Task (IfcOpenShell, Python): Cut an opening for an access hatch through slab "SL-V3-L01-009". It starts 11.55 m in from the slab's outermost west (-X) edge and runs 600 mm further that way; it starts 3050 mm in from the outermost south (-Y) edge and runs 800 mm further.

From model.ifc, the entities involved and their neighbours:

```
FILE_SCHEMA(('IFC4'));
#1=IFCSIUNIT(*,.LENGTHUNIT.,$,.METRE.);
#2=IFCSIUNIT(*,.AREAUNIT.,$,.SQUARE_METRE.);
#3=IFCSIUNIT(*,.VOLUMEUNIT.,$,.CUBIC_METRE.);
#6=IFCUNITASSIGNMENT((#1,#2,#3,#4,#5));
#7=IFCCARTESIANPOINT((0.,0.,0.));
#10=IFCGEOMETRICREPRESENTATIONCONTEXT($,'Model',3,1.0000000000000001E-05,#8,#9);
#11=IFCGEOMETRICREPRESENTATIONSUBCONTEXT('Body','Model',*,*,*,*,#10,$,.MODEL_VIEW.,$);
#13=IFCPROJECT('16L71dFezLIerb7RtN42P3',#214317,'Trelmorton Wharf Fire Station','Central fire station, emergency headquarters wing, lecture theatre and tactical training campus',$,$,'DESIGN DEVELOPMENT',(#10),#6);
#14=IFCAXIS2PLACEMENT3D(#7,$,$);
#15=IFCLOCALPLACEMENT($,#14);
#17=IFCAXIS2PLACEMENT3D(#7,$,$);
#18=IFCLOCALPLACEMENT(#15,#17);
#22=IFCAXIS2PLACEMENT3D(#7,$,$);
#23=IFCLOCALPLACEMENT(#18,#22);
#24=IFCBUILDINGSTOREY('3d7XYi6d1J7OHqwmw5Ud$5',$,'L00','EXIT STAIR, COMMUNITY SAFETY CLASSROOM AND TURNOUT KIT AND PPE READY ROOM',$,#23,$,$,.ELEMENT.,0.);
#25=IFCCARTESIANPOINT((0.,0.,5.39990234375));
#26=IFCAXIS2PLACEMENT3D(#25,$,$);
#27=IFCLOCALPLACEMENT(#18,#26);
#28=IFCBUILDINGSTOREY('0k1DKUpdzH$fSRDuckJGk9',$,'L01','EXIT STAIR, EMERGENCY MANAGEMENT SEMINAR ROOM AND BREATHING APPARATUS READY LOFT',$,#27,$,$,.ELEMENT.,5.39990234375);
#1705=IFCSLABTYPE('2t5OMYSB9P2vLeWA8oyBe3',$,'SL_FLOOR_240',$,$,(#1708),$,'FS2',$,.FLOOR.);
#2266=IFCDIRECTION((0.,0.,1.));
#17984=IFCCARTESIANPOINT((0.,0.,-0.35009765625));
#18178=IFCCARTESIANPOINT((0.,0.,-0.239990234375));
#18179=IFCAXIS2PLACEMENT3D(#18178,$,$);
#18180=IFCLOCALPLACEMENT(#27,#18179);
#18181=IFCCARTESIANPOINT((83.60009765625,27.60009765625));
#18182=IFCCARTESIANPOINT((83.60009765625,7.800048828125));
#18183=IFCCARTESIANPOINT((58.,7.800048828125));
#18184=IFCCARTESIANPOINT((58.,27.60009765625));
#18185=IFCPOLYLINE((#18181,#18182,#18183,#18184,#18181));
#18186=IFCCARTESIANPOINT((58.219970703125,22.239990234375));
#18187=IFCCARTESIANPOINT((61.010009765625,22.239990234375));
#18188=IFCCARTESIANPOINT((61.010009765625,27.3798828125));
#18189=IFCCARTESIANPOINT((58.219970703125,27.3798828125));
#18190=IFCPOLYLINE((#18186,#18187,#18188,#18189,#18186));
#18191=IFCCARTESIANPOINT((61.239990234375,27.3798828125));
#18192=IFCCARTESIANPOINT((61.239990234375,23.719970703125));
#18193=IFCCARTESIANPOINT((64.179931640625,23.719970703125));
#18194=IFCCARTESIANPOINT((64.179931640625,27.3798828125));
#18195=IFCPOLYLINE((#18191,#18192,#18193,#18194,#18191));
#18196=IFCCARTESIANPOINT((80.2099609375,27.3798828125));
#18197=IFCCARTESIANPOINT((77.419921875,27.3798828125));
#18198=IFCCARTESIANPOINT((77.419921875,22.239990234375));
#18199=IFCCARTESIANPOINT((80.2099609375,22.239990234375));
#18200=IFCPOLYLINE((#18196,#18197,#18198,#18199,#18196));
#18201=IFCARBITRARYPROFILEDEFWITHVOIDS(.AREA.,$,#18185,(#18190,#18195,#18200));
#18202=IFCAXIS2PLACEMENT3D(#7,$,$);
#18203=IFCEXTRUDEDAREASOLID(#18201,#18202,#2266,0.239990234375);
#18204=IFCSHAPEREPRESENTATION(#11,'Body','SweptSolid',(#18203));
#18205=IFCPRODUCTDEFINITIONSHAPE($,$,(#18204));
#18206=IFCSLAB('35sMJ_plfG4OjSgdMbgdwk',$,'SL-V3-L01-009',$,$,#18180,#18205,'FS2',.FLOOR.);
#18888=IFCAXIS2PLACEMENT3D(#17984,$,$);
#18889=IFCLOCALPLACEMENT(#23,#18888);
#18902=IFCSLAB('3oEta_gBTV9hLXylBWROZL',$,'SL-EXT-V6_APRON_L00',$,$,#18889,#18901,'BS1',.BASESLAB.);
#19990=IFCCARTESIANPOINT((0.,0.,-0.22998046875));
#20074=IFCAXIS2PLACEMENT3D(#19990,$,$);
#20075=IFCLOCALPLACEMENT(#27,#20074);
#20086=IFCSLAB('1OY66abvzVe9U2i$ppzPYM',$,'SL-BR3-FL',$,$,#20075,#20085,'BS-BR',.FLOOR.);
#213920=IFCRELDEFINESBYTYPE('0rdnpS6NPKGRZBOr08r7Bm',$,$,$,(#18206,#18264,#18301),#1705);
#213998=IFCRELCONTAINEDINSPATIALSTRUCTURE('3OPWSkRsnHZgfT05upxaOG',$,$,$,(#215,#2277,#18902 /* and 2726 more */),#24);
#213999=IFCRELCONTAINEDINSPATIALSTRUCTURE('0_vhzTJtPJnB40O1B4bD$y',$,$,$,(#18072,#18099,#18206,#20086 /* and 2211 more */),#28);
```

```python
import numpy as np
import ifcopenshell
import ifcopenshell.api.feature
import ifcopenshell.api.geometry
import ifcopenshell.api.root
import ifcopenshell.geom
import ifcopenshell.util.placement
import ifcopenshell.util.representation
import ifcopenshell.util.shape
import ifcopenshell.util.unit

model = ifcopenshell.open("model.ifc")
unit_scale = ifcopenshell.util.unit.calculate_unit_scale(model)
settings = ifcopenshell.geom.settings()


def volume(element):
    """Net volume in cubic metres, openings subtracted."""
    shape = ifcopenshell.geom.create_shape(settings, element)
    return ifcopenshell.util.shape.get_volume(shape.geometry)


slab = model.by_id(18206)
before = volume(slab)

# Extent in the slab's own axes, in metres. The edges named are its -X and -Y sides.
slab_shape = ifcopenshell.geom.create_shape(settings, slab)
vertices = ifcopenshell.util.shape.get_vertices(slab_shape.geometry)
x_min, y_min, bottom = vertices.min(axis=0)
top = vertices[:, 2].max()

opening = ifcopenshell.api.root.create_entity(model, ifc_class="IfcOpeningElement", name="Access hatch opening", predefined_type="OPENING")
context = ifcopenshell.util.representation.get_context(model, "Model", "Body", "MODEL_VIEW")
width, depth = 0.6, 0.8
outline = [(0.0, 0.0), (width, 0.0), (width, depth), (0.0, depth), (0.0, 0.0)]
# Overshoot both faces by 50 mm so the cut is clean.
shape = ifcopenshell.api.geometry.add_slab_representation(
    model, context=context, depth=top - bottom + 0.1, polyline=outline
)
ifcopenshell.api.geometry.assign_representation(model, product=opening, representation=shape)

matrix = ifcopenshell.util.placement.get_local_placement(slab.ObjectPlacement)
matrix[:, 3] = matrix @ np.append(np.array([x_min + 11.55, y_min + 3.05, bottom - 0.05]) / unit_scale, 1.0)
ifcopenshell.api.geometry.edit_object_placement(model, product=opening, matrix=matrix, is_si=False)
ifcopenshell.api.feature.add_feature(model, feature=opening, element=slab)

after = volume(slab)

print(f"slab volume {before:.3f} -> {after:.3f} m3")

model.write("model_updated.ifc")
```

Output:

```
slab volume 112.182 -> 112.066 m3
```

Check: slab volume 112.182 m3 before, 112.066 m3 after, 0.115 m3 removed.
